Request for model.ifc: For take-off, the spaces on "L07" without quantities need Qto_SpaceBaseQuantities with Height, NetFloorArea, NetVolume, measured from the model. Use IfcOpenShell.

First a look at what the model holds.

```python
import ifcopenshell
import ifcopenshell.util.element
import ifcopenshell.util.unit

model = ifcopenshell.open("model.ifc")
print(model.schema)
for unit_type in ("LENGTHUNIT", "AREAUNIT", "VOLUMEUNIT"):
    print(unit_type, ifcopenshell.util.unit.calculate_unit_scale(model, unit_type))
storey = next(s for s in model.by_type("IfcBuildingStorey") if s.Name == "L07")
spaces = [e for e in ifcopenshell.util.element.get_decomposition(storey) if e.is_a("IfcSpace")]
for e in sorted(spaces, key=lambda e: e.id()):
    print(e.id(), e.is_a(), e.Name, list(ifcopenshell.util.element.get_psets(e, qtos_only=True)), sep=" | ")
```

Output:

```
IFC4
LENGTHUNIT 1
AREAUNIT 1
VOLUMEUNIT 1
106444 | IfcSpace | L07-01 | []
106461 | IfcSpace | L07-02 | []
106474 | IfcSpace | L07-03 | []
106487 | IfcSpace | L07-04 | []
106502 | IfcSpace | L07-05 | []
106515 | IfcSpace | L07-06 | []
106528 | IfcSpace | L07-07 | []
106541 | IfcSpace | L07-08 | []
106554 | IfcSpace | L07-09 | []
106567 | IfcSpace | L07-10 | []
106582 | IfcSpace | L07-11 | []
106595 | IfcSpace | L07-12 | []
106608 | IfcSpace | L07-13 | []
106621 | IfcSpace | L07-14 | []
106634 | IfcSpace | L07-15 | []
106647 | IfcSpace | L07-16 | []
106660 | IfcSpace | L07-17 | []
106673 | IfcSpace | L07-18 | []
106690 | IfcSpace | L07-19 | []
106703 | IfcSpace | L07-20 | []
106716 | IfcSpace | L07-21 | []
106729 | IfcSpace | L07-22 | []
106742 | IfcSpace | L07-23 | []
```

```python
import ifcopenshell
import ifcopenshell.api.pset
import ifcopenshell.geom
import ifcopenshell.util.element
import ifcopenshell.util.shape
import ifcopenshell.util.unit

model = ifcopenshell.open("model.ifc")
unit_scale = ifcopenshell.util.unit.calculate_unit_scale(model)
area_scale = ifcopenshell.util.unit.calculate_unit_scale(model, "AREAUNIT")
volume_scale = ifcopenshell.util.unit.calculate_unit_scale(model, "VOLUMEUNIT")
settings = ifcopenshell.geom.settings()

storey = next(s for s in model.by_type("IfcBuildingStorey") if s.Name == "L07")
spaces = [e for e in ifcopenshell.util.element.get_decomposition(storey) if e.is_a("IfcSpace")]

for e in sorted(spaces, key=lambda e: e.id()):
    if ifcopenshell.util.element.get_psets(e, qtos_only=True, should_inherit=False):
        continue
    # Geometry comes back in metres, in the element's own axes.
    shape = ifcopenshell.geom.create_shape(settings, e)
    values = {
        "Height": ifcopenshell.util.shape.get_z(shape.geometry) / unit_scale,
        "NetFloorArea": ifcopenshell.util.shape.get_footprint_area(shape.geometry) / area_scale,
        "NetVolume": ifcopenshell.util.shape.get_volume(shape.geometry) / volume_scale,
    }
    qto = ifcopenshell.api.pset.add_qto(model, product=e, name="Qto_SpaceBaseQuantities")
    ifcopenshell.api.pset.edit_qto(model, qto=qto, properties=values)
    print(e.id(), {k: round(v, 3) for k, v in values.items()})

model.write("model_edited.ifc")
```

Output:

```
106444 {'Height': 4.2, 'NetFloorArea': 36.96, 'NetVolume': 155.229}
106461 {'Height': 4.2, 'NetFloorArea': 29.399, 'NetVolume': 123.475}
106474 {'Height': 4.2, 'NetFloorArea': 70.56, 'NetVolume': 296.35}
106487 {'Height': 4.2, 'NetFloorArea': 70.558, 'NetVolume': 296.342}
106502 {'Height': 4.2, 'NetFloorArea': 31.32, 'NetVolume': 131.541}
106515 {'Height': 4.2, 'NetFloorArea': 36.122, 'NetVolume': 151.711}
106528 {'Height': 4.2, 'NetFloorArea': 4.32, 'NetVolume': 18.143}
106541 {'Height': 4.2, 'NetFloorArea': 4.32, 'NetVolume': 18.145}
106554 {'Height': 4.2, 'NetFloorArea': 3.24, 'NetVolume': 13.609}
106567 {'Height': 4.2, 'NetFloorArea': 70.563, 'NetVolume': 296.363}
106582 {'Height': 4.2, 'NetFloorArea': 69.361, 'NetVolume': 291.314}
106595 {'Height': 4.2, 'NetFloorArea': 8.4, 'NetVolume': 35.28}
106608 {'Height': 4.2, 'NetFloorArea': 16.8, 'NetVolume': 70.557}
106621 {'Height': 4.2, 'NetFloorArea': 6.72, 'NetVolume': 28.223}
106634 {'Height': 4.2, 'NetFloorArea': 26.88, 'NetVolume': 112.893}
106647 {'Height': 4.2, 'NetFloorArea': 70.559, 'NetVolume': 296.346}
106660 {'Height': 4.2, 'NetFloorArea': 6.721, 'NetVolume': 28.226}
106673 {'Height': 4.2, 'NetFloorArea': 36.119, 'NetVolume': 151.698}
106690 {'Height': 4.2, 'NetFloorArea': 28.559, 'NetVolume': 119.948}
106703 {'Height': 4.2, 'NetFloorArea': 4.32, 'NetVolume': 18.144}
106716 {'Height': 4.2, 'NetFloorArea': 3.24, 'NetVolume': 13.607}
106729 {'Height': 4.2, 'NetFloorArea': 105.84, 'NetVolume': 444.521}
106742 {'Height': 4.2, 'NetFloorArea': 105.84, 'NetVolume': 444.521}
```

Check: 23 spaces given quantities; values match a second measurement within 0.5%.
